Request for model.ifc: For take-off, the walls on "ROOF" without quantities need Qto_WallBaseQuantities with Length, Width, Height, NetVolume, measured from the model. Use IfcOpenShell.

First a look at what the model holds.

```python
import ifcopenshell
import ifcopenshell.util.element
import ifcopenshell.util.unit

model = ifcopenshell.open("model.ifc")
print(model.schema)
for unit_type in ("LENGTHUNIT", "AREAUNIT", "VOLUMEUNIT"):
    print(unit_type, ifcopenshell.util.unit.calculate_unit_scale(model, unit_type))
storey = next(s for s in model.by_type("IfcBuildingStorey") if s.Name == "ROOF")
walls = [e for e in ifcopenshell.util.element.get_decomposition(storey) if e.is_a("IfcWall")]
for e in sorted(walls, key=lambda e: e.id()):
    print(e.id(), e.is_a(), e.Name, list(ifcopenshell.util.element.get_psets(e, qtos_only=True)), sep=" | ")
```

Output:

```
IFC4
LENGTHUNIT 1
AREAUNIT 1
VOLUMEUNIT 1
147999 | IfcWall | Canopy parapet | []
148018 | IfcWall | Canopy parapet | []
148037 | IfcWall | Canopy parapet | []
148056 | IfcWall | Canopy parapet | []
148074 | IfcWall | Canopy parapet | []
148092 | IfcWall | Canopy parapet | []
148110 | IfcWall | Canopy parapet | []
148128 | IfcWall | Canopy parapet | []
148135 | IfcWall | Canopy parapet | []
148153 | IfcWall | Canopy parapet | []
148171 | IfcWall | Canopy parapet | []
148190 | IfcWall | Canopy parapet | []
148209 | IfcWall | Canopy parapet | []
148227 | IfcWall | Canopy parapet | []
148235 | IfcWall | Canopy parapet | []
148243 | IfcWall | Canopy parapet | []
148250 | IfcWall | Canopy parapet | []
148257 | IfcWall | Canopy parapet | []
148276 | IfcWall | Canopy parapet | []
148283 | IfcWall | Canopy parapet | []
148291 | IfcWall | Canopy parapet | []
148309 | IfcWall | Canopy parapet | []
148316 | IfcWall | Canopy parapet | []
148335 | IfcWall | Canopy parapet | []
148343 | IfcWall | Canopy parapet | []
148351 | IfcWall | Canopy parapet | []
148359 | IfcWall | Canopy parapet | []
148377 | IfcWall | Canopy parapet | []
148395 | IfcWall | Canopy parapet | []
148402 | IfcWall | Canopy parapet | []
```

```python
import ifcopenshell
import ifcopenshell.api.pset
import ifcopenshell.geom
import ifcopenshell.util.element
import ifcopenshell.util.shape
import ifcopenshell.util.unit

model = ifcopenshell.open("model.ifc")
unit_scale = ifcopenshell.util.unit.calculate_unit_scale(model)
volume_scale = ifcopenshell.util.unit.calculate_unit_scale(model, "VOLUMEUNIT")
settings = ifcopenshell.geom.settings()

storey = next(s for s in model.by_type("IfcBuildingStorey") if s.Name == "ROOF")
walls = [e for e in ifcopenshell.util.element.get_decomposition(storey) if e.is_a("IfcWall")]

for e in sorted(walls, key=lambda e: e.id()):
    if ifcopenshell.util.element.get_psets(e, qtos_only=True, should_inherit=False):
        continue
    # Geometry comes back in metres, in the element's own axes.
    shape = ifcopenshell.geom.create_shape(settings, e)
    values = {
        "Length": ifcopenshell.util.shape.get_x(shape.geometry) / unit_scale,
        "Width": ifcopenshell.util.shape.get_y(shape.geometry) / unit_scale,
        "Height": ifcopenshell.util.shape.get_z(shape.geometry) / unit_scale,
        "NetVolume": ifcopenshell.util.shape.get_volume(shape.geometry) / volume_scale,
    }
    qto = ifcopenshell.api.pset.add_qto(model, product=e, name="Qto_WallBaseQuantities")
    ifcopenshell.api.pset.edit_qto(model, qto=qto, properties=values)
    print(e.id(), {k: round(v, 3) for k, v in values.items()})

model.write("model_updated.ifc")
```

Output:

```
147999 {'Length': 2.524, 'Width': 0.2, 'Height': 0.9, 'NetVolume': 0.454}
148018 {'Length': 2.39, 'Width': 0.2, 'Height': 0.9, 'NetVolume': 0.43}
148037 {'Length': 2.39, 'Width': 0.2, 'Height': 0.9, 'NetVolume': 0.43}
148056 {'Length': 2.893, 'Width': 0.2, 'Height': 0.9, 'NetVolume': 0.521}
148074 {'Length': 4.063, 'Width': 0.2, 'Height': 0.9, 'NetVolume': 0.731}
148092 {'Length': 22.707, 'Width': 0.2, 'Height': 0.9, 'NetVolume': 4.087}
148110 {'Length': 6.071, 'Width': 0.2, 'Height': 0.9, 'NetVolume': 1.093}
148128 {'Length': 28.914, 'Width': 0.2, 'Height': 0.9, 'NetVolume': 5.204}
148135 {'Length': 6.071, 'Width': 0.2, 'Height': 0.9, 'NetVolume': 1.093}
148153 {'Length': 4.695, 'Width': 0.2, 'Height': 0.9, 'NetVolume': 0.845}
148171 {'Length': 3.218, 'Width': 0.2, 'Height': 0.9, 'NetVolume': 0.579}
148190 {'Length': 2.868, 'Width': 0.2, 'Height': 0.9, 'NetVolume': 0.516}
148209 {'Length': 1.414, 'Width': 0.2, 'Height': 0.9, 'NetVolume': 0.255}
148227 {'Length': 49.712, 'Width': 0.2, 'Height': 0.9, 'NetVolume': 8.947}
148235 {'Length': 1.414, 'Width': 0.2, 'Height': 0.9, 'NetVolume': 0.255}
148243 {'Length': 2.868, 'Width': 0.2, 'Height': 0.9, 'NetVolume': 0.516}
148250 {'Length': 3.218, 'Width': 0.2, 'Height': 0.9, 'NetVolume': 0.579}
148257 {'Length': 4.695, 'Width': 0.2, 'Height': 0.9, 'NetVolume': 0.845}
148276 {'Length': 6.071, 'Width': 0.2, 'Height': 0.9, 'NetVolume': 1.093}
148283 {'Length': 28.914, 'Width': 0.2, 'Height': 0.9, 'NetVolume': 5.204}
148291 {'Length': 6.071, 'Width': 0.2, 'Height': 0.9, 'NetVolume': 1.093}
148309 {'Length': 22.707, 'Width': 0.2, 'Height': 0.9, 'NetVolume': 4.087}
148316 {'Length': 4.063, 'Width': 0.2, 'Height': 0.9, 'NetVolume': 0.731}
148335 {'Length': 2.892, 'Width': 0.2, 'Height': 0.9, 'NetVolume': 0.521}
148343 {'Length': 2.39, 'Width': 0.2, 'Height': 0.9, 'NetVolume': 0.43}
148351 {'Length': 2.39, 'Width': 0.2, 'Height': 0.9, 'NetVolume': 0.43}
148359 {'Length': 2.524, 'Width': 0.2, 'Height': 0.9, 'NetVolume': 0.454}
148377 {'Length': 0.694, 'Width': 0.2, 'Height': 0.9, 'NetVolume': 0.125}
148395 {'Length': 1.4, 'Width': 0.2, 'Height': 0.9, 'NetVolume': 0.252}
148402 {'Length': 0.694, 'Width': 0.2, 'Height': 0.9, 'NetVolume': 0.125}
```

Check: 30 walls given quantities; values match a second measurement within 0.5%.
